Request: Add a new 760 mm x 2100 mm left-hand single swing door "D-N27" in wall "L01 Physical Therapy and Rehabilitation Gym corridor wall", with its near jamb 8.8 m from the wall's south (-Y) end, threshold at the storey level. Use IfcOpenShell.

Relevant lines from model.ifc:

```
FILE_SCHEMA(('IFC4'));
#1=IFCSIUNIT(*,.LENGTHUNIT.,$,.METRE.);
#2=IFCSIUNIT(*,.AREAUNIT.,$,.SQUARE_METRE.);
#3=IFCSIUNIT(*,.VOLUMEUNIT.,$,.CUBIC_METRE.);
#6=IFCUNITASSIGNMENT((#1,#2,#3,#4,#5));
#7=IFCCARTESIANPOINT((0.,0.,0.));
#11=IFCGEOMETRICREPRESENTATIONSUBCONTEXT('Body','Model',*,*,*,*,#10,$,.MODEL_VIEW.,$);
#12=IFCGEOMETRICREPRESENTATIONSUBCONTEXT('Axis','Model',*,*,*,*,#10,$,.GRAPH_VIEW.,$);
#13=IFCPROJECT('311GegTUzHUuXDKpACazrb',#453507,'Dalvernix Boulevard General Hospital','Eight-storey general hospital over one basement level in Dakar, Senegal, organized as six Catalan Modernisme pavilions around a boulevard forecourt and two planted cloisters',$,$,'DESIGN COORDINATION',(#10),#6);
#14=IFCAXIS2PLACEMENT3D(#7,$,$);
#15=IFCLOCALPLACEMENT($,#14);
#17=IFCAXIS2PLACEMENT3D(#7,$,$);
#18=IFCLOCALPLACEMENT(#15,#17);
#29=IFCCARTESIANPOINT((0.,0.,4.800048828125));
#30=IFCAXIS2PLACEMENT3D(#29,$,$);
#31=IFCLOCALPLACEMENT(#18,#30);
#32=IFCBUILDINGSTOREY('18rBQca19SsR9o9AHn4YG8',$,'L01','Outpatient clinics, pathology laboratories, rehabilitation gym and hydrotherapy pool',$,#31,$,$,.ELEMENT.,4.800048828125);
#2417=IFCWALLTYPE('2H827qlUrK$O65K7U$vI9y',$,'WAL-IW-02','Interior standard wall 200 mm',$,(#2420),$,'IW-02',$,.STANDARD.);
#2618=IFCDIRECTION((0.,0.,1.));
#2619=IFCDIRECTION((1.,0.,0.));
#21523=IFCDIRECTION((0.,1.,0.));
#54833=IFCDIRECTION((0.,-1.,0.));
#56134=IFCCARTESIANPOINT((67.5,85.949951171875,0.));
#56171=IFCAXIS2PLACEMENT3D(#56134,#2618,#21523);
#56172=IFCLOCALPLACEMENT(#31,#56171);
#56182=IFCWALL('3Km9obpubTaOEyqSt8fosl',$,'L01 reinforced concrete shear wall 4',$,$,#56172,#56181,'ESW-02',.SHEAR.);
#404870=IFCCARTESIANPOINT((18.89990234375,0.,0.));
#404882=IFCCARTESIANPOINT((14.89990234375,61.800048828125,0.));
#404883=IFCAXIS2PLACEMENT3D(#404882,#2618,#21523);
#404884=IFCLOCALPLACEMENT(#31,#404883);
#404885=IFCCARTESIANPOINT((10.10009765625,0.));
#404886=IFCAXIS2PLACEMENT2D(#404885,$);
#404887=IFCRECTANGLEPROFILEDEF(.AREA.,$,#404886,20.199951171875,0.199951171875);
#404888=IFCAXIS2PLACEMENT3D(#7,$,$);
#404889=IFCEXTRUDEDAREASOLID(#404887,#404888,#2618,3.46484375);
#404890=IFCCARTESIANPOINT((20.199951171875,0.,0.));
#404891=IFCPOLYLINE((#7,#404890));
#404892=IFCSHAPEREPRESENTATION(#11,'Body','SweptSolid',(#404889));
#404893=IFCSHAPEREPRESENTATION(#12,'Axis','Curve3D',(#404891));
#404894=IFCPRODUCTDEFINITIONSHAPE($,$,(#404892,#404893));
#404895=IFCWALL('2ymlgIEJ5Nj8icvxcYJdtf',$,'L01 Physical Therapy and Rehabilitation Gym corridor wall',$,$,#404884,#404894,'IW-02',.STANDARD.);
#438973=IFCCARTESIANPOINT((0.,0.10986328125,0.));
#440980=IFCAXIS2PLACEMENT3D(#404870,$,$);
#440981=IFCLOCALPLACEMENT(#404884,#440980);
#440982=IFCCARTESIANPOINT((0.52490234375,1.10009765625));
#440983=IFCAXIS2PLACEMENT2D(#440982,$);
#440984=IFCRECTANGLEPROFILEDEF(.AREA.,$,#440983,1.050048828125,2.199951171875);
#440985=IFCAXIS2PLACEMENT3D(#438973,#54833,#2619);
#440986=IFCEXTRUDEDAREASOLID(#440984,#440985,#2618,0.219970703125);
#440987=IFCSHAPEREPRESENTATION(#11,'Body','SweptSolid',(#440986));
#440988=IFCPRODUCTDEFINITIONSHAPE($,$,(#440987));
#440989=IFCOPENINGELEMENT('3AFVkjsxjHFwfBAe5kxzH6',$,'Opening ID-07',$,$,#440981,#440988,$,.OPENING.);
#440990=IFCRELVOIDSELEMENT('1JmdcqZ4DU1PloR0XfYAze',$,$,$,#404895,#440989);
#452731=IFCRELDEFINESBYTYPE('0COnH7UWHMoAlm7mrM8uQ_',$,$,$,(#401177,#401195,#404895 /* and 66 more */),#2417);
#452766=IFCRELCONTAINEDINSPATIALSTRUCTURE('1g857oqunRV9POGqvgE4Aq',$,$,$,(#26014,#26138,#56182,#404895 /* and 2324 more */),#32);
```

```python
import numpy as np
import ifcopenshell
import ifcopenshell.api.feature
import ifcopenshell.api.geometry
import ifcopenshell.api.root
import ifcopenshell.api.spatial
import ifcopenshell.geom
import ifcopenshell.util.element
import ifcopenshell.util.placement
import ifcopenshell.util.representation
import ifcopenshell.util.shape
import ifcopenshell.util.unit

model = ifcopenshell.open("model.ifc")
unit_scale = ifcopenshell.util.unit.calculate_unit_scale(model)
settings = ifcopenshell.geom.settings()


def volume(element):
    """Net volume in cubic metres, openings subtracted."""
    shape = ifcopenshell.geom.create_shape(settings, element)
    return ifcopenshell.util.shape.get_volume(shape.geometry)


wall = model.by_guid("2ymlgIEJ5Nj8icvxcYJdtf")
storey = ifcopenshell.util.element.get_container(wall, ifc_class="IfcBuildingStorey")
context = ifcopenshell.util.representation.get_context(model, "Model", "Body", "MODEL_VIEW")
before = volume(wall)

width, height, from_end, sill = 0.76, 2.1, 8.8, 0.0  # metres

# The wall runs along its own X axis, and the end named is its -X end.
wall_shape = ifcopenshell.geom.create_shape(settings, wall)
x, y, z = ifcopenshell.util.shape.get_vertices(wall_shape.geometry).T
start = x.min() + from_end
face, thickness = float(y.min()), float(y.max() - y.min())
wall_matrix = ifcopenshell.util.placement.get_local_placement(wall.ObjectPlacement)
level = ifcopenshell.util.placement.get_local_placement(storey.ObjectPlacement)[2, 3]


def in_wall(x, y):
    """Placement at x, y metres in the wall's axes, at sill height."""
    matrix = wall_matrix.copy()
    matrix[:, 3] = wall_matrix @ np.array([x / unit_scale, y / unit_scale, 0.0, 1.0])
    matrix[2, 3] = level + sill / unit_scale
    return matrix


# Opening: a box that overshoots both wall faces by 50 mm.
opening = ifcopenshell.api.root.create_entity(model, ifc_class="IfcOpeningElement", predefined_type="OPENING")
box = ifcopenshell.api.geometry.add_wall_representation(
    model, context=context, length=width, height=height, thickness=thickness + 0.1
)
ifcopenshell.api.geometry.assign_representation(model, product=opening, representation=box)
ifcopenshell.api.geometry.edit_object_placement(model, product=opening, matrix=in_wall(start, face - 0.05), is_si=False)
ifcopenshell.api.feature.add_feature(model, feature=opening, element=wall)

door = ifcopenshell.api.root.create_entity(model, ifc_class="IfcDoor", name="D-N27", predefined_type="DOOR")
door.OverallWidth, door.OverallHeight = width / unit_scale, height / unit_scale
door.OperationType = "SINGLE_SWING_LEFT"
body = ifcopenshell.api.geometry.add_door_representation(
    model,
    context=context,
    overall_width=door.OverallWidth,
    overall_height=door.OverallHeight,
    operation_type="SINGLE_SWING_LEFT",
    lining_properties={"LiningDepth": thickness / unit_scale, "ThresholdDepth": thickness / unit_scale},
)
ifcopenshell.api.geometry.assign_representation(model, product=door, representation=body)
ifcopenshell.api.spatial.assign_container(model, products=[door], relating_structure=storey)
ifcopenshell.api.feature.add_filling(model, opening=opening, element=door)

# The lining spans the wall, so the door starts at the wall face.
ifcopenshell.api.geometry.edit_object_placement(model, product=door, matrix=in_wall(start, face), is_si=False)

after = volume(wall)

print(f"wall volume {before:.3f} -> {after:.3f} m3")

model.write("model_rev.ifc")
```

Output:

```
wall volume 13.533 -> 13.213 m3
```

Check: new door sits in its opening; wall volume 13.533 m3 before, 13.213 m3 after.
